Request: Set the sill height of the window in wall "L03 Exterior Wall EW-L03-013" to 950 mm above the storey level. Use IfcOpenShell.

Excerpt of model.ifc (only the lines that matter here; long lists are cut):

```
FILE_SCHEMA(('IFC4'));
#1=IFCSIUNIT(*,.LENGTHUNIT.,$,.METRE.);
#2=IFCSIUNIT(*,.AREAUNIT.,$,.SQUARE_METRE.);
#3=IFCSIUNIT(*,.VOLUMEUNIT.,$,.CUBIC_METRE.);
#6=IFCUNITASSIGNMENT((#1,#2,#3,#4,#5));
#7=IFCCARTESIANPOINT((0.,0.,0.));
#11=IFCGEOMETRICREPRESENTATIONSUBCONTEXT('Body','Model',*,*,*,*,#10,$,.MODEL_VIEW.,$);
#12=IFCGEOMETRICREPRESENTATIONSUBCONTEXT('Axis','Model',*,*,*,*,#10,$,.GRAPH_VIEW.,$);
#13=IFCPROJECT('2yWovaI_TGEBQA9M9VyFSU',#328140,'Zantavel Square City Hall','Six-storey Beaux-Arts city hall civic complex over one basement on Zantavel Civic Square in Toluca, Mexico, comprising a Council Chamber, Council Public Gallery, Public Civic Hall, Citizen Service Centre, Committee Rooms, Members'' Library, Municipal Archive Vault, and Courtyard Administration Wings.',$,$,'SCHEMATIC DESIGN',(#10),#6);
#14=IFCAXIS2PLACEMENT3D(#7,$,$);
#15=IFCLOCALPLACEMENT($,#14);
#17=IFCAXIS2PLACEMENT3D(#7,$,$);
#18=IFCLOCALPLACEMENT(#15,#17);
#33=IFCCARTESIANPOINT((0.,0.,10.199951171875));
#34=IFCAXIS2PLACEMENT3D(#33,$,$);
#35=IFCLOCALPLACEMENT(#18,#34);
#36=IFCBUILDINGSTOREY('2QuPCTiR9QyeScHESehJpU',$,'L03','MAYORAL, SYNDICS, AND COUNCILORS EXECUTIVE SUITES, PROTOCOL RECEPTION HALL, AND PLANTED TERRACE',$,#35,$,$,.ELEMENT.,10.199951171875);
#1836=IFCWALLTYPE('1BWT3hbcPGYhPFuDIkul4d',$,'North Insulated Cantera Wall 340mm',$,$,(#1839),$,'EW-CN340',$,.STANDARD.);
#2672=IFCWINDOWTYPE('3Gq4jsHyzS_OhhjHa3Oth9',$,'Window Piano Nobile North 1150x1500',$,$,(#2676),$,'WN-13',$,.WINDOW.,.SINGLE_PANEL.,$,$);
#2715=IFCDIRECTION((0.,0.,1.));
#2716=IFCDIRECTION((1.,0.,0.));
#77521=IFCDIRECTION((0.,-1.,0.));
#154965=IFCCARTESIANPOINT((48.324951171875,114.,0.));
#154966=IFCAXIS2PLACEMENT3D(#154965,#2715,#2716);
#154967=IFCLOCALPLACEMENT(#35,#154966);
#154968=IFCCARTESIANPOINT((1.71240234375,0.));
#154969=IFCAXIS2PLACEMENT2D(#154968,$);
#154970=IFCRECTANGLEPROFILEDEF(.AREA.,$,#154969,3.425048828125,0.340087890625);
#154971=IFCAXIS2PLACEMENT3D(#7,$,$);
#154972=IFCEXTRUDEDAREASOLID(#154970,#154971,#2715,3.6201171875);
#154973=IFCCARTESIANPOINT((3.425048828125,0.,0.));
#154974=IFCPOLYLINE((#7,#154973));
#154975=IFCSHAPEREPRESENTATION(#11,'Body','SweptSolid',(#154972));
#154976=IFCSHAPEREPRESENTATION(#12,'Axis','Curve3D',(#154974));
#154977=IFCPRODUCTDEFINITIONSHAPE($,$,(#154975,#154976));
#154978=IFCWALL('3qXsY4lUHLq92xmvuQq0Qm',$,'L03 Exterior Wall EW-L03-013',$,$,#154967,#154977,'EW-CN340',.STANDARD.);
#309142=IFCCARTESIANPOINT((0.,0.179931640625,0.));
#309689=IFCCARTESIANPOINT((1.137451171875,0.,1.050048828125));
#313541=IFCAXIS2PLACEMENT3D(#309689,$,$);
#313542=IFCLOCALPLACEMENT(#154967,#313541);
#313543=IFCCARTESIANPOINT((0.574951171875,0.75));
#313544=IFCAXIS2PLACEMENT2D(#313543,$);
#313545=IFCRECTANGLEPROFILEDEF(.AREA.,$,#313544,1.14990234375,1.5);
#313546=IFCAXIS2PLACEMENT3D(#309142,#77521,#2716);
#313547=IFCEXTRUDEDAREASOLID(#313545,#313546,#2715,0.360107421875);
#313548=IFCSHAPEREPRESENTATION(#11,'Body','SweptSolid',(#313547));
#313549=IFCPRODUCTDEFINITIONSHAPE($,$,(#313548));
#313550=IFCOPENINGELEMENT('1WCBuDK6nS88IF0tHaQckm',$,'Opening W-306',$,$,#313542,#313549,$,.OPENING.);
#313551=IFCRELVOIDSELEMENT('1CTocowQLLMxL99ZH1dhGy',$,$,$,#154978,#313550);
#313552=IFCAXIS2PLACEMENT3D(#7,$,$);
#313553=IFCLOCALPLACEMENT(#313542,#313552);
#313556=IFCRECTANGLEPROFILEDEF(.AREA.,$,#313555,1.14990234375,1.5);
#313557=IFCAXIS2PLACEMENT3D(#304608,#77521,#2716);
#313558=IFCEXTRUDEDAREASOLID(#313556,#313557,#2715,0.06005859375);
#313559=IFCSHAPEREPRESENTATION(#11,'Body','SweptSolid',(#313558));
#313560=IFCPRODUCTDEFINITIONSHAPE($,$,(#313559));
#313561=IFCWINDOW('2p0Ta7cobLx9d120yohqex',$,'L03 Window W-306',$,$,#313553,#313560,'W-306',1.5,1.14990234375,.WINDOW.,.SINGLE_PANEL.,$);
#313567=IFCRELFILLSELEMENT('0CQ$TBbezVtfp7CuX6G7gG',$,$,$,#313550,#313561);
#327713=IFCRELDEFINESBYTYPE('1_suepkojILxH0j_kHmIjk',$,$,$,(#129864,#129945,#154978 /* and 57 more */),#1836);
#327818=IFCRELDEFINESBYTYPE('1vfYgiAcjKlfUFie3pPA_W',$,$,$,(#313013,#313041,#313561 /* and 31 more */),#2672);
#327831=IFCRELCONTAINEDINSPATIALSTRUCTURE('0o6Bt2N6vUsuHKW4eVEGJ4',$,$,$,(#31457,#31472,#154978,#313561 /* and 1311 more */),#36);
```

```python
import numpy as np
import ifcopenshell
import ifcopenshell.api.geometry
import ifcopenshell.geom
import ifcopenshell.util.element
import ifcopenshell.util.placement
import ifcopenshell.util.shape
import ifcopenshell.util.unit

model = ifcopenshell.open("model.ifc")
unit_scale = ifcopenshell.util.unit.calculate_unit_scale(model)

window = model.by_id(313561)
opening = window.FillsVoids[0].RelatingOpeningElement
storey = ifcopenshell.util.element.get_container(window, ifc_class="IfcBuildingStorey")
level = ifcopenshell.util.placement.get_local_placement(storey.ObjectPlacement)[2, 3]

# The opening's origin need not be at the sill, so measure its lowest point.
shape = ifcopenshell.geom.create_shape(ifcopenshell.geom.settings(), opening)
bottom = ifcopenshell.util.shape.get_shape_bottom_elevation(shape, shape.geometry) / unit_scale
dz = level + 0.95 / unit_scale - bottom

shift = np.array([0.0, 0.0, dz])
# The window is placed relative to its opening, so it follows when the opening moves.
matrix = ifcopenshell.util.placement.get_local_placement(opening.ObjectPlacement)
matrix[:3, 3] += shift
ifcopenshell.api.geometry.edit_object_placement(
    model, product=opening, matrix=matrix, is_si=False, should_transform_children=True
)

print(f"moved by {dz * unit_scale:+.3f} m")

model.write("model-out.ifc")
```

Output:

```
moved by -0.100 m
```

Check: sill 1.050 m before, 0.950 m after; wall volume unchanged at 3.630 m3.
